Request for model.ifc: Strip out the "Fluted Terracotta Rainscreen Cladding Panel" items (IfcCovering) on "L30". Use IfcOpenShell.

First a look at what the model holds.

```python
import ifcopenshell
import ifcopenshell.util.element

model = ifcopenshell.open("model.ifc")
print(model.schema)
storey = next(s for s in model.by_type("IfcBuildingStorey") if s.Name == "L30")
coverings = [e for e in ifcopenshell.util.element.get_decomposition(storey) if e.is_a("IfcCovering")]
seen = {}
for e in coverings:
    element_type = ifcopenshell.util.element.get_type(e)
    name = element_type.Name if element_type not in (None, e) else None
    seen[name] = seen.get(name, 0) + 1
for name, count in sorted(seen.items(), key=str):
    print(count, "x", name)
```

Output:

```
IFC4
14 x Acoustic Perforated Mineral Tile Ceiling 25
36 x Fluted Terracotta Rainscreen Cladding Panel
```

```python
import ifcopenshell
import ifcopenshell.api.root
import ifcopenshell.util.element

model = ifcopenshell.open("model.ifc")

storey = next(s for s in model.by_type("IfcBuildingStorey") if s.Name == "L30")
coverings = [e for e in ifcopenshell.util.element.get_decomposition(storey) if e.is_a("IfcCovering")]
targets = [e for e in coverings if (t := ifcopenshell.util.element.get_type(e)) not in (None, e) and t.Name == "Fluted Terracotta Rainscreen Cladding Panel"]

for e in targets:
    ifcopenshell.api.root.remove_product(model, product=e)
print(len(targets), "removed")

model.write("model_updated.ifc")
```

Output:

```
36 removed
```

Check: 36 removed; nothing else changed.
